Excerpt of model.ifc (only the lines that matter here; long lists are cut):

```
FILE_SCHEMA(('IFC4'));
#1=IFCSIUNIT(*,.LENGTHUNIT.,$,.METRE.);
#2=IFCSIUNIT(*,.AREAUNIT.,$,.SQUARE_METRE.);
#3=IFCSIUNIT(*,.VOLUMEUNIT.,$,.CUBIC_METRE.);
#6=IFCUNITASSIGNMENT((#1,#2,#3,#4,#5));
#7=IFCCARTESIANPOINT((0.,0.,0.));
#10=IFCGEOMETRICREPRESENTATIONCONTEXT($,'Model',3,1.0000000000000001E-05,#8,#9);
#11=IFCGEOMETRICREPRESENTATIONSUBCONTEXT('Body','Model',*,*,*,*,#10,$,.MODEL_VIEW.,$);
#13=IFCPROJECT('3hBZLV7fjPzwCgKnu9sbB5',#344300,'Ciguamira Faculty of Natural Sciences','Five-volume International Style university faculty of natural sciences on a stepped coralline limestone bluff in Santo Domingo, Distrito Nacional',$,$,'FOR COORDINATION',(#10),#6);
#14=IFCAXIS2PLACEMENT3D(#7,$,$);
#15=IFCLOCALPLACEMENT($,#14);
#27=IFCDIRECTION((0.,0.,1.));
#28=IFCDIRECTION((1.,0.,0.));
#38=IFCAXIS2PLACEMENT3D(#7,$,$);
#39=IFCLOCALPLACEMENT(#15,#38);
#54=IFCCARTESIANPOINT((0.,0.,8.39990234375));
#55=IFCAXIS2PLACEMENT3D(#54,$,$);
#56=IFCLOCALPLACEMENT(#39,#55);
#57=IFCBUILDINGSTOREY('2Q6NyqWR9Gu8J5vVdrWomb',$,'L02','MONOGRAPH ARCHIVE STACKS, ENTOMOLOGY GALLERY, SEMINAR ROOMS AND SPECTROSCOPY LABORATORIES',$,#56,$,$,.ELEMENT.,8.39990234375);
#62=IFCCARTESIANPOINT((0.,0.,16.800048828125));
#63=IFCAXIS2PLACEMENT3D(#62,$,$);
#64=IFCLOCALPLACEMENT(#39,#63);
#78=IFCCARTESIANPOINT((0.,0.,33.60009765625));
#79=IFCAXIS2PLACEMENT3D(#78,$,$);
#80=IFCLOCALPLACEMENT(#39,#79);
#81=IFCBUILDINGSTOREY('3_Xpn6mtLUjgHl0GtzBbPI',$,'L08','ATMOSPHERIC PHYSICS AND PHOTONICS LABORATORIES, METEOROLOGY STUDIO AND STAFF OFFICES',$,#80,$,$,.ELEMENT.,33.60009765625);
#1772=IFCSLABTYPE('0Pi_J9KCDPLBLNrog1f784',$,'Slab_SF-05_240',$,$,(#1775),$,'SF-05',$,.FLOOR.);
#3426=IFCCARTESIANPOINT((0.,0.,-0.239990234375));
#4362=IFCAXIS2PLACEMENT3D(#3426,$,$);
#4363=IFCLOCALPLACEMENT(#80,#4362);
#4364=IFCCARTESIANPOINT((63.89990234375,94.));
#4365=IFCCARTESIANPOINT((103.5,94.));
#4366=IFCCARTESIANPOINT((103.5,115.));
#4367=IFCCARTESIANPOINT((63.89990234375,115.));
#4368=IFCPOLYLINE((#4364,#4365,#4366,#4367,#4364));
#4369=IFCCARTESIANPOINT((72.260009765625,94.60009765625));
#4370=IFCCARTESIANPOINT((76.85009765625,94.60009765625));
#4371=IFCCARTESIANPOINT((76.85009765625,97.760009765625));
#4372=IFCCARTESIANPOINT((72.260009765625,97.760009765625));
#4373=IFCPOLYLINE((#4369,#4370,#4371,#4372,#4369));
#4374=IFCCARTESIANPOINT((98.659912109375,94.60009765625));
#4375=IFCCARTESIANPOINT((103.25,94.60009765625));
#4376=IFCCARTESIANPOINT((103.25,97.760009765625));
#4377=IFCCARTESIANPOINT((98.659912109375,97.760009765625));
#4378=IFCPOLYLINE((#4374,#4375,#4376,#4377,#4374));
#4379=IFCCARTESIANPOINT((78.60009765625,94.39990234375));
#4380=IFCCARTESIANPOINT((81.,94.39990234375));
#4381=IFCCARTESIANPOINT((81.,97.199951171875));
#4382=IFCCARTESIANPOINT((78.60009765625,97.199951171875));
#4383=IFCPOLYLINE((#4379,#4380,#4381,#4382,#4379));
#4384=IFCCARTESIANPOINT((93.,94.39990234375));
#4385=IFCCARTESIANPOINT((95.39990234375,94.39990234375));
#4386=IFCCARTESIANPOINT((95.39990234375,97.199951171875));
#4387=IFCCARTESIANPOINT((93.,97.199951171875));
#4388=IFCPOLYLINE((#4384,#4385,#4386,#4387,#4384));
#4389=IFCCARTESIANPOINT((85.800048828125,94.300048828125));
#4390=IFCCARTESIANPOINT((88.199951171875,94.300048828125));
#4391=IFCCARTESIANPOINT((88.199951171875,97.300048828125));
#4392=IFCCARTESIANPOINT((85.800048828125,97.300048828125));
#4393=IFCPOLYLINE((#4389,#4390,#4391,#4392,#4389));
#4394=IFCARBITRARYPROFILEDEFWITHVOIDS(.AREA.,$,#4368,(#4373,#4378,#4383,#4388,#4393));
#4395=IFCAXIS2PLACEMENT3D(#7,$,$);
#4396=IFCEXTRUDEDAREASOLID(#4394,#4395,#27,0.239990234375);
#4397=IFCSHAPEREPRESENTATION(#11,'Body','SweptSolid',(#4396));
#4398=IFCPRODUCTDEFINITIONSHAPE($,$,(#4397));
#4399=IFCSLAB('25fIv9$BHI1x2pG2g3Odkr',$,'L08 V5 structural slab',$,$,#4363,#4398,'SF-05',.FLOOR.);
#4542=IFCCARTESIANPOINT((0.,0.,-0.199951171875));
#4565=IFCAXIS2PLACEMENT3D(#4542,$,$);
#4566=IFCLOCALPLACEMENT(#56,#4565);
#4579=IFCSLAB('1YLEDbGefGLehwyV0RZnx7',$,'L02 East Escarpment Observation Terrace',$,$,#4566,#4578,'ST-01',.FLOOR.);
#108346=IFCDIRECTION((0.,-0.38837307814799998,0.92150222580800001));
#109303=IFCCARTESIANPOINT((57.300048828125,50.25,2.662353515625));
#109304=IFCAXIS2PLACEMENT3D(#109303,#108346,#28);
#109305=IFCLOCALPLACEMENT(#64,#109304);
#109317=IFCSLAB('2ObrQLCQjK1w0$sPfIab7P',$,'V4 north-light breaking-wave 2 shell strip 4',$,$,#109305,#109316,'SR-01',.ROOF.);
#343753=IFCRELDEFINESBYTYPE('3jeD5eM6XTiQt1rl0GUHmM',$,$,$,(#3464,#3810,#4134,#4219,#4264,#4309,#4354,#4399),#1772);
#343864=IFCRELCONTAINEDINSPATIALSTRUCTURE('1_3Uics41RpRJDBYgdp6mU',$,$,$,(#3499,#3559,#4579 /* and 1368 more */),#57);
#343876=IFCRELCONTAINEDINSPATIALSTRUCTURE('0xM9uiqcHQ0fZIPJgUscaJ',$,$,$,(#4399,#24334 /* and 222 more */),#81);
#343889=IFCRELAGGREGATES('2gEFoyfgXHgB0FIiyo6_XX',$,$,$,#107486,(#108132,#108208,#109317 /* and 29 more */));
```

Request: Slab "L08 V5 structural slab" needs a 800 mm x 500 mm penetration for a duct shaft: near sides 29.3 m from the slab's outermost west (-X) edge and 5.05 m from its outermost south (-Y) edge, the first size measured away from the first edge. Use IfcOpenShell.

```python
import numpy as np
import ifcopenshell
import ifcopenshell.api.feature
import ifcopenshell.api.geometry
import ifcopenshell.api.root
import ifcopenshell.geom
import ifcopenshell.util.placement
import ifcopenshell.util.representation
import ifcopenshell.util.shape
import ifcopenshell.util.unit

model = ifcopenshell.open("model.ifc")
unit_scale = ifcopenshell.util.unit.calculate_unit_scale(model)
settings = ifcopenshell.geom.settings()


def volume(element):
    """Net volume in cubic metres, openings subtracted."""
    shape = ifcopenshell.geom.create_shape(settings, element)
    return ifcopenshell.util.shape.get_volume(shape.geometry)


slab = model.by_id(4399)
before = volume(slab)

# Extent in the slab's own axes, in metres. The edges named are its -X and -Y sides.
slab_shape = ifcopenshell.geom.create_shape(settings, slab)
vertices = ifcopenshell.util.shape.get_vertices(slab_shape.geometry)
x_min, y_min, bottom = vertices.min(axis=0)
top = vertices[:, 2].max()

opening = ifcopenshell.api.root.create_entity(model, ifc_class="IfcOpeningElement", name="Duct shaft opening", predefined_type="OPENING")
context = ifcopenshell.util.representation.get_context(model, "Model", "Body", "MODEL_VIEW")
width, depth = 0.8, 0.5
outline = [(0.0, 0.0), (width, 0.0), (width, depth), (0.0, depth), (0.0, 0.0)]
# Overshoot both faces by 50 mm so the cut is clean.
shape = ifcopenshell.api.geometry.add_slab_representation(
    model, context=context, depth=top - bottom + 0.1, polyline=outline
)
ifcopenshell.api.geometry.assign_representation(model, product=opening, representation=shape)

matrix = ifcopenshell.util.placement.get_local_placement(slab.ObjectPlacement)
matrix[:, 3] = matrix @ np.append(np.array([x_min + 29.3, y_min + 5.05, bottom - 0.05]) / unit_scale, 1.0)
ifcopenshell.api.geometry.edit_object_placement(model, product=opening, matrix=matrix, is_si=False)
ifcopenshell.api.feature.add_feature(model, feature=opening, element=slab)

after = volume(slab)

print(f"slab volume {before:.3f} -> {after:.3f} m3")

model.write("model_v2.ifc")
```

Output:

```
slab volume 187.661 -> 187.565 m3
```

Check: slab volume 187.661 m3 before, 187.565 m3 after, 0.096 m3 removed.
